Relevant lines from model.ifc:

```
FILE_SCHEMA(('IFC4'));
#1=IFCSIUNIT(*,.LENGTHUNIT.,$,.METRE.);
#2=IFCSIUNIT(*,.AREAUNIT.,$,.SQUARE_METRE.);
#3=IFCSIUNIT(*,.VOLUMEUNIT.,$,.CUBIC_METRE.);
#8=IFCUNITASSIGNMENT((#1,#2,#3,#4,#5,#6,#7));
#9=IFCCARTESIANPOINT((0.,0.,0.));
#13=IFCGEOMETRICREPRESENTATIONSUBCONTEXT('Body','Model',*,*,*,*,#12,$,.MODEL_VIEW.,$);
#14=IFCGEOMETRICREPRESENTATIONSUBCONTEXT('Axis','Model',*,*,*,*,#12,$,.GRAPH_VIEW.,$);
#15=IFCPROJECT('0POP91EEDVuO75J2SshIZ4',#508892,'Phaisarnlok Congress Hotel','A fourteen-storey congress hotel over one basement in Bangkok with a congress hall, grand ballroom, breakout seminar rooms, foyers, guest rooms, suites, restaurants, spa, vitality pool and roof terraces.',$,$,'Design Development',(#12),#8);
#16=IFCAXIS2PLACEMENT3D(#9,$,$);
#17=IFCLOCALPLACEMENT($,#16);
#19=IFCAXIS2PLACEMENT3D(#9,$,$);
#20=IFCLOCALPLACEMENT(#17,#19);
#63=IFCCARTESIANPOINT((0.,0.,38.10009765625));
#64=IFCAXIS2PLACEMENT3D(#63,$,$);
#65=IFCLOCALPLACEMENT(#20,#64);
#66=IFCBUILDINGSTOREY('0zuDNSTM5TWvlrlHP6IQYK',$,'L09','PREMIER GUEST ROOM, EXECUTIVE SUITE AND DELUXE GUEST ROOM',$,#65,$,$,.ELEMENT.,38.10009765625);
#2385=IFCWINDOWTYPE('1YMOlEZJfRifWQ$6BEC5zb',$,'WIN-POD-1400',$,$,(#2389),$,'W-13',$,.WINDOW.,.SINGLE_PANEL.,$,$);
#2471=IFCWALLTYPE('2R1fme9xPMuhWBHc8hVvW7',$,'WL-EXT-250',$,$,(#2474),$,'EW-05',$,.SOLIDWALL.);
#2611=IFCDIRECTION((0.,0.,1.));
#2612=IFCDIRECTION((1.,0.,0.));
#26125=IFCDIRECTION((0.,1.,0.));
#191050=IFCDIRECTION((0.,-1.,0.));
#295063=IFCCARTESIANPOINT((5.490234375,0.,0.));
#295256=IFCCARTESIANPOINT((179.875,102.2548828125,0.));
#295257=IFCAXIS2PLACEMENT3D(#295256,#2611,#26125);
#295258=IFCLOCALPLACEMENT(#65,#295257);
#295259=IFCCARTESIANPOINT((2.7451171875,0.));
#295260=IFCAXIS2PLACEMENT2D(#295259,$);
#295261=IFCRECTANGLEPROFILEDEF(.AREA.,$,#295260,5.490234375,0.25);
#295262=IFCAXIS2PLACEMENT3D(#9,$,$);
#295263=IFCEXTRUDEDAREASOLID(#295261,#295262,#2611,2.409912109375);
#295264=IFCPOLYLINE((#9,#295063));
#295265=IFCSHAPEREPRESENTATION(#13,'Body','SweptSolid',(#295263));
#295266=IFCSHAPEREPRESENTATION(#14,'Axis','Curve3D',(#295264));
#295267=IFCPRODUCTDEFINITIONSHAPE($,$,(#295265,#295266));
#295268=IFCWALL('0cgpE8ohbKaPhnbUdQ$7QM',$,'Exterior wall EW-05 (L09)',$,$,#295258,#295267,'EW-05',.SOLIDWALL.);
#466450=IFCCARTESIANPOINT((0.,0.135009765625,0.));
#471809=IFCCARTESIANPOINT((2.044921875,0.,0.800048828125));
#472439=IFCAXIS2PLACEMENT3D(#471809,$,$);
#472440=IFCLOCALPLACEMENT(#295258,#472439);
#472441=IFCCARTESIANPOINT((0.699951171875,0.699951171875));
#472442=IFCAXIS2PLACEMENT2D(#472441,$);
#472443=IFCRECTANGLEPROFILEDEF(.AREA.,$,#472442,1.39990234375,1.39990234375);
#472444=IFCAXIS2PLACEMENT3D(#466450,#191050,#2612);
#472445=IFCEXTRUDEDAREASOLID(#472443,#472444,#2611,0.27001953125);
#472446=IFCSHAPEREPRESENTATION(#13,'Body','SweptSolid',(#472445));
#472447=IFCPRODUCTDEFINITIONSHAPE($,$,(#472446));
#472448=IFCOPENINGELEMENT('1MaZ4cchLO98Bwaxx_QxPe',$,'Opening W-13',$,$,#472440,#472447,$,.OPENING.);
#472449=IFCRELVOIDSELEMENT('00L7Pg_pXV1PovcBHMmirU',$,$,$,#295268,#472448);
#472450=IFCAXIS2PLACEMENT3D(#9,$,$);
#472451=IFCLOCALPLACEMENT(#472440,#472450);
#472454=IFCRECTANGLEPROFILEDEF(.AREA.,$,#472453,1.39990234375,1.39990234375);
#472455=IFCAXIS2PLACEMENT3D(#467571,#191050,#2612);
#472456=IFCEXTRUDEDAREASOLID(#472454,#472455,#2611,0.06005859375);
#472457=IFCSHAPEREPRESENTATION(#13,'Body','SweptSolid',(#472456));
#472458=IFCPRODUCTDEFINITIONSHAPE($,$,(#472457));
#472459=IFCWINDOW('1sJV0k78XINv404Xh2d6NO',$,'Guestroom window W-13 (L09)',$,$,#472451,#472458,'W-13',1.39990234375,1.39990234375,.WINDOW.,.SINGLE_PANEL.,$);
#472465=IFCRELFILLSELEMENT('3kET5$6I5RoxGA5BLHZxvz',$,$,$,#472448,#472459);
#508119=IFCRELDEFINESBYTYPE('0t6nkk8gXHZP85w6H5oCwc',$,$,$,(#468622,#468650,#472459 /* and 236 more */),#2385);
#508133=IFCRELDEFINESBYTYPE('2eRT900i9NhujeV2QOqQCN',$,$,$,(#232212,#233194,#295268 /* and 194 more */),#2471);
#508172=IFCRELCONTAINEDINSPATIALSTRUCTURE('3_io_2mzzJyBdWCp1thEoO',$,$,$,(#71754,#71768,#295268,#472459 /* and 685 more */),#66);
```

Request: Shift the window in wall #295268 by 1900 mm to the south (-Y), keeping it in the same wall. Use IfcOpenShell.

```python
import ifcopenshell
import ifcopenshell.api.geometry
import ifcopenshell.util.placement
import ifcopenshell.util.unit

model = ifcopenshell.open("model.ifc")
unit_scale = ifcopenshell.util.unit.calculate_unit_scale(model)

window = model.by_guid("1sJV0k78XINv404Xh2d6NO")
opening = window.FillsVoids[0].RelatingOpeningElement
wall = opening.VoidsElements[0].RelatingBuildingElement

wall_matrix = ifcopenshell.util.placement.get_local_placement(wall.ObjectPlacement)
shift = wall_matrix[:3, 0] * -1.9 / unit_scale
before = ifcopenshell.util.placement.get_local_placement(window.ObjectPlacement)[:3, 3].copy()

# The window is placed relative to its opening, so it follows when the opening moves.
matrix = ifcopenshell.util.placement.get_local_placement(opening.ObjectPlacement)
matrix[:3, 3] += shift
ifcopenshell.api.geometry.edit_object_placement(
    model, product=opening, matrix=matrix, is_si=False, should_transform_children=True
)

after = ifcopenshell.util.placement.get_local_placement(window.ObjectPlacement)[:3, 3]
print("window moved by", (after - before).round(3) + 0.0)

model.write("model_rev.ifc")
```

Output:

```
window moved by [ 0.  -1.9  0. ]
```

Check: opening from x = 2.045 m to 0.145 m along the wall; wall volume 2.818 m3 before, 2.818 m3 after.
